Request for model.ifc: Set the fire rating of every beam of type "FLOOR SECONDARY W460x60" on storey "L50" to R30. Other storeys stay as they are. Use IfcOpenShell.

First a look at what the model holds.

```python
import ifcopenshell
import ifcopenshell.util.element

model = ifcopenshell.open("model.ifc")
print(model.schema)
storey = next(s for s in model.by_type("IfcBuildingStorey") if s.Name == "L50")
beams = [e for e in ifcopenshell.util.element.get_decomposition(storey) if e.is_a("IfcBeam")]
seen = {}
for e in beams:
    element_type = ifcopenshell.util.element.get_type(e)
    key = (element_type.Name if element_type != e and element_type else None, ifcopenshell.util.element.get_pset(e, "Pset_BeamCommon", "FireRating"))
    seen[key] = seen.get(key, 0) + 1
for (name, value), count in sorted(seen.items(), key=str):
    print(count, "x", name, "|", value)
```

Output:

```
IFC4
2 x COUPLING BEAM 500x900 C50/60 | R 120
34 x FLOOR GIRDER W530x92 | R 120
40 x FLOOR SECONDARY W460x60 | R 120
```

```python
import ifcopenshell
import ifcopenshell.api.pset
import ifcopenshell.util.element

model = ifcopenshell.open("model.ifc")

storey = next(s for s in model.by_type("IfcBuildingStorey") if s.Name == "L50")
beams = [e for e in ifcopenshell.util.element.get_decomposition(storey) if e.is_a("IfcBeam")]

count = 0
for e in beams:
    element_type = ifcopenshell.util.element.get_type(e)
    if element_type in (None, e) or element_type.Name != "FLOOR SECONDARY W460x60":
        continue
    found = ifcopenshell.util.element.get_pset(e, "Pset_BeamCommon", should_inherit=False)
    if found:
        pset = model.by_id(found["id"])
        if len(ifcopenshell.util.element.get_elements_by_pset(pset)) > 1:
            pset = ifcopenshell.api.pset.unshare_pset(model, products=[e], pset=pset)[0]
    else:
        pset = ifcopenshell.api.pset.add_pset(model, product=e, name="Pset_BeamCommon")
    ifcopenshell.api.pset.edit_pset(model, pset=pset, properties={"FireRating": "R30"})
    count += 1

print(count, "beams updated")

model.write("model_rev.ifc")
```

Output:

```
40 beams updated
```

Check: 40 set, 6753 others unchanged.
